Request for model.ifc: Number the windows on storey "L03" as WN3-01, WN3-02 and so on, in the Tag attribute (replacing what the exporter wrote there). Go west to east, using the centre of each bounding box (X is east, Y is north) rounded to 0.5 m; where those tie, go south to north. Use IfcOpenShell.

First a look at what the model holds.

```python
import ifcopenshell
import ifcopenshell.util.element
import ifcopenshell.util.placement

model = ifcopenshell.open("model.ifc")
print(model.schema)
storey = next(s for s in model.by_type("IfcBuildingStorey") if s.Name == "L03")
windows = [e for e in ifcopenshell.util.element.get_decomposition(storey) if e.is_a("IfcWindow")]
for e in sorted(windows, key=lambda e: e.id()):
    origin = ifcopenshell.util.placement.get_local_placement(e.ObjectPlacement)[:3, 3]
    print(e.id(), e.Tag, e.Name, origin.round(2) + 0.0, sep=" | ")
```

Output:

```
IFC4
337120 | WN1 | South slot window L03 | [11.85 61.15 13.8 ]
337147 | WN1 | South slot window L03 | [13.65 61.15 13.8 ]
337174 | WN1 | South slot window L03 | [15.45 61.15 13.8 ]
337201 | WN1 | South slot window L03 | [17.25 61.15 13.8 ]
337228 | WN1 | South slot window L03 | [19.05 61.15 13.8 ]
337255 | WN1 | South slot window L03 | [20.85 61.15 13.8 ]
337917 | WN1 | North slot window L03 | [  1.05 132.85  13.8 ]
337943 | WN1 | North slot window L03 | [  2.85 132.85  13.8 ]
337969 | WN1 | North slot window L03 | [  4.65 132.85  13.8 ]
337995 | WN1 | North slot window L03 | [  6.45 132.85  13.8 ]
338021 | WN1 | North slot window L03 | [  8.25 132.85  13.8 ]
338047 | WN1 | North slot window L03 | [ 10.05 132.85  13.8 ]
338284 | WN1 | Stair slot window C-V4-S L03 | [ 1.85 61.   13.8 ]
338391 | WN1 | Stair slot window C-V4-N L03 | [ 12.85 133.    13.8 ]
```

```python
import ifcopenshell
import ifcopenshell.geom
import ifcopenshell.util.element
import ifcopenshell.util.shape

model = ifcopenshell.open("model.ifc")
settings = ifcopenshell.geom.settings()
settings.set("use-world-coords", True)


def centre(element):
    shape = ifcopenshell.geom.create_shape(settings, element)
    return ifcopenshell.util.shape.get_bbox_centroid(shape.geometry)


storey = next(s for s in model.by_type("IfcBuildingStorey") if s.Name == "L03")
windows = [e for e in ifcopenshell.util.element.get_decomposition(storey) if e.is_a("IfcWindow")]

# Insertion points can sit at a corner or the storey origin, so sort by the geometry (in metres).
centres = {e: centre(e) for e in windows}
windows.sort(key=lambda e: (round(centres[e][0] / 0.5), centres[e][1]))

for i, e in enumerate(windows, start=1):
    number = f"WN3-{i:02d}"
    e.Tag = number
    print(e.id(), number)

model.write("model_updated.ifc")
```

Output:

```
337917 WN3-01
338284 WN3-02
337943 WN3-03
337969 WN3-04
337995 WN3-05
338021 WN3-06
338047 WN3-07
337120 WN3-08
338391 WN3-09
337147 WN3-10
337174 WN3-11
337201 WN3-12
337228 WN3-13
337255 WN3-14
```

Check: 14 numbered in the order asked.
